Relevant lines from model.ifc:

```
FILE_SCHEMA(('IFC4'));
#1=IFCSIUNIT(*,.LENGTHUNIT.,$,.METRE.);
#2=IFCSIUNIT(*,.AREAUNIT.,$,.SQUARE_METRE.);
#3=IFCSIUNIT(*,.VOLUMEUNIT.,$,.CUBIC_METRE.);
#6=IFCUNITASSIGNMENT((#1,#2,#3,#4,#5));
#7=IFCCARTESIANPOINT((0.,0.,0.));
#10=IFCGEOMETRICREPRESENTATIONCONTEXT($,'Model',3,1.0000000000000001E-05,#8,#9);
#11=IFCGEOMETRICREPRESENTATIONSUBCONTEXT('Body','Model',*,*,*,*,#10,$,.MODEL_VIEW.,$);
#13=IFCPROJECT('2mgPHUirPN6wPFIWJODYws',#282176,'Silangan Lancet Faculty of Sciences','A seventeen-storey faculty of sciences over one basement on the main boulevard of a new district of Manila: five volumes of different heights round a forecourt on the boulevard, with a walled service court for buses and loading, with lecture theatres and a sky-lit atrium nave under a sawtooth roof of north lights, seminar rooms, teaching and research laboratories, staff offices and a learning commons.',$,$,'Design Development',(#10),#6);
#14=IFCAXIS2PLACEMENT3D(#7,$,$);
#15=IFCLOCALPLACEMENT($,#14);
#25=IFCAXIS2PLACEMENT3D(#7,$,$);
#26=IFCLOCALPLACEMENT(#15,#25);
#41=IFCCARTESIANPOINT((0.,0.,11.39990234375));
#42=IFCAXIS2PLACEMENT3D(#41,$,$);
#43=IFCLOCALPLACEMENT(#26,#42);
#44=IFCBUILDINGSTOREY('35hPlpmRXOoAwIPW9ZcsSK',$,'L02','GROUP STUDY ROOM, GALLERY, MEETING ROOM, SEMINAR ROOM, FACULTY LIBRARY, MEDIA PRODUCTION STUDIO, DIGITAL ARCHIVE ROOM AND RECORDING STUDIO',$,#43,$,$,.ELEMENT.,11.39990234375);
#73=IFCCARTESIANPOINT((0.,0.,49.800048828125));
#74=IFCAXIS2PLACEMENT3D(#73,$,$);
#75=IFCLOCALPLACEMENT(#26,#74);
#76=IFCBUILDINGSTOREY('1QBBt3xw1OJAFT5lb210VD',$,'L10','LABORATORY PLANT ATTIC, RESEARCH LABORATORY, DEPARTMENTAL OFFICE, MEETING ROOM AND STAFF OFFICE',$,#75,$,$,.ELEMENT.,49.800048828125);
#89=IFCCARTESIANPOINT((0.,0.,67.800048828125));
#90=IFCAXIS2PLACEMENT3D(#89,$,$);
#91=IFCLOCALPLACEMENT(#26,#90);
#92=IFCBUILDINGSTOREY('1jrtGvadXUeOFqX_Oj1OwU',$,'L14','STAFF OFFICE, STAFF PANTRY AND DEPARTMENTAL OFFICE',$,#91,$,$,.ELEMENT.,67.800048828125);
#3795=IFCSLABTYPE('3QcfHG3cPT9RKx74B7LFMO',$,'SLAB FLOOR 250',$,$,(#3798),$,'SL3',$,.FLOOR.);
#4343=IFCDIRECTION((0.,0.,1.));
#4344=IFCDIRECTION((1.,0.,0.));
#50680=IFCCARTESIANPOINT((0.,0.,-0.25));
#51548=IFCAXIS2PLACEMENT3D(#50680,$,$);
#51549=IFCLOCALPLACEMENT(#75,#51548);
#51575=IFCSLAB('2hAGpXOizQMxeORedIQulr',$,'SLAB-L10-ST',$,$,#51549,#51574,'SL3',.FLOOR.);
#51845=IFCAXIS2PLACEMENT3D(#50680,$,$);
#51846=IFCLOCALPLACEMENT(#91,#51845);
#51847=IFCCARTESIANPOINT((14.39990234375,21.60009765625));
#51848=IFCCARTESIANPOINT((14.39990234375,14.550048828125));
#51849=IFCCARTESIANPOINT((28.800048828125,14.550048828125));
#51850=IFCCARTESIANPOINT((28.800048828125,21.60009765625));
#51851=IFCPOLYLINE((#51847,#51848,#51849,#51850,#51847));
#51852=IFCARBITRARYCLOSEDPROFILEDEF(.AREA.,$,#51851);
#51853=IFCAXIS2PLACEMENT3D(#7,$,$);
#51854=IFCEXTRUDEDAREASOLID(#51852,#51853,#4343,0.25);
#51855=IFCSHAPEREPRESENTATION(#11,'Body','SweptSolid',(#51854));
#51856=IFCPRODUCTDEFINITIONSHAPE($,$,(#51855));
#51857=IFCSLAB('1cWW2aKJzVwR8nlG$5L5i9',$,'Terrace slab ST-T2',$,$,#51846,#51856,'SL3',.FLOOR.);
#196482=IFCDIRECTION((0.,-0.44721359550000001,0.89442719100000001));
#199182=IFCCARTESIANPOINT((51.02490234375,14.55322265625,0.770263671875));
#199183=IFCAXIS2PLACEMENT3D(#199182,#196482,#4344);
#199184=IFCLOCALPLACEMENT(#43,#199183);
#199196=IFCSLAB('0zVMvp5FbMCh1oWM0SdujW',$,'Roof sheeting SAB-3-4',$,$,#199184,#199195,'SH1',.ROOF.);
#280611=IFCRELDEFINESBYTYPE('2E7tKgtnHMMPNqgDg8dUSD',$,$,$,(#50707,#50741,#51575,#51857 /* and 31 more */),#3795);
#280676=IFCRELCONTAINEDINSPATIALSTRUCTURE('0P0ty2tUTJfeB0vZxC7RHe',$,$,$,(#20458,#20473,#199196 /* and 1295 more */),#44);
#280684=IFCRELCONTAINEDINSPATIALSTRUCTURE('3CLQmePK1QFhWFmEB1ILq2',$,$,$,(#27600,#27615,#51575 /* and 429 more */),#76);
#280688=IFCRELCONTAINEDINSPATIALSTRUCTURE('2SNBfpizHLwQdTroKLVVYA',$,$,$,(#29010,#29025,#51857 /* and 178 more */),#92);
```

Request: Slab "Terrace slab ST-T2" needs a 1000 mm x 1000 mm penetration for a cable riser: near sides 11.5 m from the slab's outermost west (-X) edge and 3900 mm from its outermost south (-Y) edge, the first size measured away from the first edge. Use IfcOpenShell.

```python
import numpy as np
import ifcopenshell
import ifcopenshell.api.feature
import ifcopenshell.api.geometry
import ifcopenshell.api.root
import ifcopenshell.geom
import ifcopenshell.util.placement
import ifcopenshell.util.representation
import ifcopenshell.util.shape
import ifcopenshell.util.unit

model = ifcopenshell.open("model.ifc")
unit_scale = ifcopenshell.util.unit.calculate_unit_scale(model)
settings = ifcopenshell.geom.settings()


def volume(element):
    """Net volume in cubic metres, openings subtracted."""
    shape = ifcopenshell.geom.create_shape(settings, element)
    return ifcopenshell.util.shape.get_volume(shape.geometry)


slab = model.by_id(51857)
before = volume(slab)

# Extent in the slab's own axes, in metres. The edges named are its -X and -Y sides.
slab_shape = ifcopenshell.geom.create_shape(settings, slab)
vertices = ifcopenshell.util.shape.get_vertices(slab_shape.geometry)
x_min, y_min, bottom = vertices.min(axis=0)
top = vertices[:, 2].max()

opening = ifcopenshell.api.root.create_entity(model, ifc_class="IfcOpeningElement", name="Cable riser opening", predefined_type="OPENING")
context = ifcopenshell.util.representation.get_context(model, "Model", "Body", "MODEL_VIEW")
width, depth = 1, 1
outline = [(0.0, 0.0), (width, 0.0), (width, depth), (0.0, depth), (0.0, 0.0)]
# Overshoot both faces by 50 mm so the cut is clean.
shape = ifcopenshell.api.geometry.add_slab_representation(
    model, context=context, depth=top - bottom + 0.1, polyline=outline
)
ifcopenshell.api.geometry.assign_representation(model, product=opening, representation=shape)

matrix = ifcopenshell.util.placement.get_local_placement(slab.ObjectPlacement)
matrix[:, 3] = matrix @ np.append(np.array([x_min + 11.5, y_min + 3.9, bottom - 0.05]) / unit_scale, 1.0)
ifcopenshell.api.geometry.edit_object_placement(model, product=opening, matrix=matrix, is_si=False)
ifcopenshell.api.feature.add_feature(model, feature=opening, element=slab)

after = volume(slab)

print(f"slab volume {before:.3f} -> {after:.3f} m3")

model.write("model-out.ifc")
```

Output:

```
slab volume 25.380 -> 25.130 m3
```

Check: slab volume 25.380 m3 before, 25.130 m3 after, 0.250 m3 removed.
